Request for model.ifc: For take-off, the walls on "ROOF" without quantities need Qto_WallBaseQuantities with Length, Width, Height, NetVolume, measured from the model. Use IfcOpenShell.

First a look at what the model holds.

```python
import ifcopenshell
import ifcopenshell.util.element
import ifcopenshell.util.unit

model = ifcopenshell.open("model.ifc")
print(model.schema)
for unit_type in ("LENGTHUNIT", "AREAUNIT", "VOLUMEUNIT"):
    print(unit_type, ifcopenshell.util.unit.calculate_unit_scale(model, unit_type))
storey = next(s for s in model.by_type("IfcBuildingStorey") if s.Name == "ROOF")
walls = [e for e in ifcopenshell.util.element.get_decomposition(storey) if e.is_a("IfcWall")]
for e in sorted(walls, key=lambda e: e.id()):
    print(e.id(), e.is_a(), e.Name, list(ifcopenshell.util.element.get_psets(e, qtos_only=True)), sep=" | ")
```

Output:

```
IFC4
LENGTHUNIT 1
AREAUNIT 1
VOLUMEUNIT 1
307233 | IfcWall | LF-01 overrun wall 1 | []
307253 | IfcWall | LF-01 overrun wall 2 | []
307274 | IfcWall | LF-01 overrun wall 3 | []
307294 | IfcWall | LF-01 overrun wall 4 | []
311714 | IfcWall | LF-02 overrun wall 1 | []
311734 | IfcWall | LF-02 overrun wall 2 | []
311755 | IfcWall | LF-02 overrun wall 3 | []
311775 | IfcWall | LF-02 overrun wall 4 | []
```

```python
import ifcopenshell
import ifcopenshell.api.pset
import ifcopenshell.geom
import ifcopenshell.util.element
import ifcopenshell.util.shape
import ifcopenshell.util.unit

model = ifcopenshell.open("model.ifc")
unit_scale = ifcopenshell.util.unit.calculate_unit_scale(model)
volume_scale = ifcopenshell.util.unit.calculate_unit_scale(model, "VOLUMEUNIT")
settings = ifcopenshell.geom.settings()

storey = next(s for s in model.by_type("IfcBuildingStorey") if s.Name == "ROOF")
walls = [e for e in ifcopenshell.util.element.get_decomposition(storey) if e.is_a("IfcWall")]

for e in sorted(walls, key=lambda e: e.id()):
    if ifcopenshell.util.element.get_psets(e, qtos_only=True, should_inherit=False):
        continue
    # Geometry comes back in metres, in the element's own axes.
    shape = ifcopenshell.geom.create_shape(settings, e)
    values = {
        "Length": ifcopenshell.util.shape.get_x(shape.geometry) / unit_scale,
        "Width": ifcopenshell.util.shape.get_y(shape.geometry) / unit_scale,
        "Height": ifcopenshell.util.shape.get_z(shape.geometry) / unit_scale,
        "NetVolume": ifcopenshell.util.shape.get_volume(shape.geometry) / volume_scale,
    }
    qto = ifcopenshell.api.pset.add_qto(model, product=e, name="Qto_WallBaseQuantities")
    ifcopenshell.api.pset.edit_qto(model, qto=qto, properties=values)
    print(e.id(), {k: round(v, 3) for k, v in values.items()})

model.write("model_edited.ifc")
```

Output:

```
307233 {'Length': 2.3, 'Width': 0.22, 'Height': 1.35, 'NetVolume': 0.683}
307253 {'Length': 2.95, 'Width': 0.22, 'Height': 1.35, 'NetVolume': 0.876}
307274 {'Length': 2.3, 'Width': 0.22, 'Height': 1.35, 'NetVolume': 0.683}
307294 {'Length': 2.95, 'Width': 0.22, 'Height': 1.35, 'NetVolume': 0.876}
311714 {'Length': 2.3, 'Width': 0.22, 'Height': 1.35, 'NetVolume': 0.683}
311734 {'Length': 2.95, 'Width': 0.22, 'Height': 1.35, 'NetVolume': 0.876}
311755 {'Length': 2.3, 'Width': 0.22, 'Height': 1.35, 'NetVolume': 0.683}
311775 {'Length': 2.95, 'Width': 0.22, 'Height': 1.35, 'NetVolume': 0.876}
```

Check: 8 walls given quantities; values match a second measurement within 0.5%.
